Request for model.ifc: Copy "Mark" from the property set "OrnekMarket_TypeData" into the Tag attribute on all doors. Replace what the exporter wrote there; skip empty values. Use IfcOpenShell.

First a look at what the model holds.

```python
import ifcopenshell
import ifcopenshell.util.element

model = ifcopenshell.open("model.ifc")
print(model.schema)
doors = model.by_type("IfcDoor")
print(len(doors), "doors")
for e in doors[:8]:
    source = ifcopenshell.util.element.get_pset(e, "OrnekMarket_TypeData", "Mark")
    target = e.Tag
    print(e.id(), repr(source), repr(target), sep=" | ")
```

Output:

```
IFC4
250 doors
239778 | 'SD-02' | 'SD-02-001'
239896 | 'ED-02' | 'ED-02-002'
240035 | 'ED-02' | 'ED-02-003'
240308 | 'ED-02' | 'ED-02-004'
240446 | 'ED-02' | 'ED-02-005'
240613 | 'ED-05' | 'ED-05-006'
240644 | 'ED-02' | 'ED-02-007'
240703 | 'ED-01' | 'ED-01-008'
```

```python
import ifcopenshell
import ifcopenshell.util.element

model = ifcopenshell.open("model.ifc")

count = 0
for e in model.by_type("IfcDoor"):
    value = ifcopenshell.util.element.get_pset(e, "OrnekMarket_TypeData", "Mark")
    current = e.Tag
    if not value or not value.strip() or current == value:
        continue
    e.Tag = value
    count += 1

print(count, "doors updated")

model.write("model_edited.ifc")
```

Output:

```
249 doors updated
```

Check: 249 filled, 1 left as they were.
